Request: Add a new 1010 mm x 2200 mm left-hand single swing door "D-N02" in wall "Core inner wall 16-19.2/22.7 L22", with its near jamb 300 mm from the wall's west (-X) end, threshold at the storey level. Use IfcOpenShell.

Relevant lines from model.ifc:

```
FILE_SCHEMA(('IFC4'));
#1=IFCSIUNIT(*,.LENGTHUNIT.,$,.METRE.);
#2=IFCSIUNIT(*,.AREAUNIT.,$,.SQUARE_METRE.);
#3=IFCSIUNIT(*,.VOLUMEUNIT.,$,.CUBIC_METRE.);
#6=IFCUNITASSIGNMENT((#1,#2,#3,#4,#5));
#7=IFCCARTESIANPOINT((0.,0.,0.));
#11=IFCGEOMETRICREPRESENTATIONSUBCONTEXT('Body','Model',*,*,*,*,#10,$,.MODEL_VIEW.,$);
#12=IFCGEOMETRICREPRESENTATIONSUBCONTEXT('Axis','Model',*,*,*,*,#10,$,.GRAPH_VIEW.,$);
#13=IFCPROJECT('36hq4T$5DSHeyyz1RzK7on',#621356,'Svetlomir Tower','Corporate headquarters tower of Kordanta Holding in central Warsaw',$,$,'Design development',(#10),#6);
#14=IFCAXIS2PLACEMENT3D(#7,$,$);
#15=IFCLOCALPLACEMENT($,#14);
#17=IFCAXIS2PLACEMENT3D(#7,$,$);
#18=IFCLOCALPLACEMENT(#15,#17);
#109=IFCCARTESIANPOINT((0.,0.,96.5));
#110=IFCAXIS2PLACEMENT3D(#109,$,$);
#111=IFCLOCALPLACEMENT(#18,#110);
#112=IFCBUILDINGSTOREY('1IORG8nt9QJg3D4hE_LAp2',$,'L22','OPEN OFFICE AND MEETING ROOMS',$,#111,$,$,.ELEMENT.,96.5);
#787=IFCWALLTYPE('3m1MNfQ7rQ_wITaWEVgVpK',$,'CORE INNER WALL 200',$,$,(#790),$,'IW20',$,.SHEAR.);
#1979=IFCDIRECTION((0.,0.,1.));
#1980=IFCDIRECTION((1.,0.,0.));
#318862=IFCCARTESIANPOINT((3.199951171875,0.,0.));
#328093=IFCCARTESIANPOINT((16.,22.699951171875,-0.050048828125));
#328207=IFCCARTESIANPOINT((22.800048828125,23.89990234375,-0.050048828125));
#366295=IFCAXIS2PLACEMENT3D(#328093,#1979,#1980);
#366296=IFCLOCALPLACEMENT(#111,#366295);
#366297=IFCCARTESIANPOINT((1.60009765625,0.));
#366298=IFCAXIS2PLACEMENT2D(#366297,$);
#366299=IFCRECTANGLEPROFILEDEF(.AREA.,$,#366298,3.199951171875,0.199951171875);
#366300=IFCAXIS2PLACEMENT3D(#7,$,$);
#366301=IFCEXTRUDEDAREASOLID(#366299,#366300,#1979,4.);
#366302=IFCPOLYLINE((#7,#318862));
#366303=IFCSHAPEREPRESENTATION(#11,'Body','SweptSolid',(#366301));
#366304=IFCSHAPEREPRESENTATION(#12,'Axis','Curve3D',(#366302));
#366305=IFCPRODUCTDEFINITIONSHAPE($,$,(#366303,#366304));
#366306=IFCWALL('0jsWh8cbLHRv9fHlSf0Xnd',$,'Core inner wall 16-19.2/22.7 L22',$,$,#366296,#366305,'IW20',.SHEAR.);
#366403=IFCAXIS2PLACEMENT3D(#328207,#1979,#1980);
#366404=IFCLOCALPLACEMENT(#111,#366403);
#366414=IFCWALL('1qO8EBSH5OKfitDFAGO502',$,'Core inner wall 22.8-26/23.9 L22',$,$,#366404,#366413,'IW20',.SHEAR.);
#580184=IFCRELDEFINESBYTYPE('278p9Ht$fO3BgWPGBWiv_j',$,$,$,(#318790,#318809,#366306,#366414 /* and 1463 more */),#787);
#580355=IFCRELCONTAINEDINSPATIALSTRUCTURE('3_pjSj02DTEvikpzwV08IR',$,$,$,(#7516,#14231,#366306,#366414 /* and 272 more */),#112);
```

```python
import numpy as np
import ifcopenshell
import ifcopenshell.api.feature
import ifcopenshell.api.geometry
import ifcopenshell.api.root
import ifcopenshell.api.spatial
import ifcopenshell.geom
import ifcopenshell.util.element
import ifcopenshell.util.placement
import ifcopenshell.util.representation
import ifcopenshell.util.shape
import ifcopenshell.util.unit

model = ifcopenshell.open("model.ifc")
unit_scale = ifcopenshell.util.unit.calculate_unit_scale(model)
settings = ifcopenshell.geom.settings()


def volume(element):
    """Net volume in cubic metres, openings subtracted."""
    shape = ifcopenshell.geom.create_shape(settings, element)
    return ifcopenshell.util.shape.get_volume(shape.geometry)


wall = model.by_guid("0jsWh8cbLHRv9fHlSf0Xnd")
storey = ifcopenshell.util.element.get_container(wall, ifc_class="IfcBuildingStorey")
context = ifcopenshell.util.representation.get_context(model, "Model", "Body", "MODEL_VIEW")
before = volume(wall)

width, height, from_end, sill = 1.01, 2.2, 0.3, 0.0  # metres

# The wall runs along its own X axis, and the end named is its -X end.
wall_shape = ifcopenshell.geom.create_shape(settings, wall)
x, y, z = ifcopenshell.util.shape.get_vertices(wall_shape.geometry).T
start = x.min() + from_end
face, thickness = float(y.min()), float(y.max() - y.min())
wall_matrix = ifcopenshell.util.placement.get_local_placement(wall.ObjectPlacement)
level = ifcopenshell.util.placement.get_local_placement(storey.ObjectPlacement)[2, 3]


def in_wall(x, y):
    """Placement at x, y metres in the wall's axes, at sill height."""
    matrix = wall_matrix.copy()
    matrix[:, 3] = wall_matrix @ np.array([x / unit_scale, y / unit_scale, 0.0, 1.0])
    matrix[2, 3] = level + sill / unit_scale
    return matrix


# Opening: a box that overshoots both wall faces by 50 mm.
opening = ifcopenshell.api.root.create_entity(model, ifc_class="IfcOpeningElement", predefined_type="OPENING")
box = ifcopenshell.api.geometry.add_wall_representation(
    model, context=context, length=width, height=height, thickness=thickness + 0.1
)
ifcopenshell.api.geometry.assign_representation(model, product=opening, representation=box)
ifcopenshell.api.geometry.edit_object_placement(model, product=opening, matrix=in_wall(start, face - 0.05), is_si=False)
ifcopenshell.api.feature.add_feature(model, feature=opening, element=wall)

door = ifcopenshell.api.root.create_entity(model, ifc_class="IfcDoor", name="D-N02", predefined_type="DOOR")
door.OverallWidth, door.OverallHeight = width / unit_scale, height / unit_scale
door.OperationType = "SINGLE_SWING_LEFT"
body = ifcopenshell.api.geometry.add_door_representation(
    model,
    context=context,
    overall_width=door.OverallWidth,
    overall_height=door.OverallHeight,
    operation_type="SINGLE_SWING_LEFT",
    lining_properties={"LiningDepth": thickness / unit_scale, "ThresholdDepth": thickness / unit_scale},
)
ifcopenshell.api.geometry.assign_representation(model, product=door, representation=body)
ifcopenshell.api.spatial.assign_container(model, products=[door], relating_structure=storey)
ifcopenshell.api.feature.add_filling(model, opening=opening, element=door)

# The lining spans the wall, so the door starts at the wall face.
ifcopenshell.api.geometry.edit_object_placement(model, product=door, matrix=in_wall(start, face), is_si=False)

after = volume(wall)

print(f"wall volume {before:.3f} -> {after:.3f} m3")

model.write("model_edited.ifc")
```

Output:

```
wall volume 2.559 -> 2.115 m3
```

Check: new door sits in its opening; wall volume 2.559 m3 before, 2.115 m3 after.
